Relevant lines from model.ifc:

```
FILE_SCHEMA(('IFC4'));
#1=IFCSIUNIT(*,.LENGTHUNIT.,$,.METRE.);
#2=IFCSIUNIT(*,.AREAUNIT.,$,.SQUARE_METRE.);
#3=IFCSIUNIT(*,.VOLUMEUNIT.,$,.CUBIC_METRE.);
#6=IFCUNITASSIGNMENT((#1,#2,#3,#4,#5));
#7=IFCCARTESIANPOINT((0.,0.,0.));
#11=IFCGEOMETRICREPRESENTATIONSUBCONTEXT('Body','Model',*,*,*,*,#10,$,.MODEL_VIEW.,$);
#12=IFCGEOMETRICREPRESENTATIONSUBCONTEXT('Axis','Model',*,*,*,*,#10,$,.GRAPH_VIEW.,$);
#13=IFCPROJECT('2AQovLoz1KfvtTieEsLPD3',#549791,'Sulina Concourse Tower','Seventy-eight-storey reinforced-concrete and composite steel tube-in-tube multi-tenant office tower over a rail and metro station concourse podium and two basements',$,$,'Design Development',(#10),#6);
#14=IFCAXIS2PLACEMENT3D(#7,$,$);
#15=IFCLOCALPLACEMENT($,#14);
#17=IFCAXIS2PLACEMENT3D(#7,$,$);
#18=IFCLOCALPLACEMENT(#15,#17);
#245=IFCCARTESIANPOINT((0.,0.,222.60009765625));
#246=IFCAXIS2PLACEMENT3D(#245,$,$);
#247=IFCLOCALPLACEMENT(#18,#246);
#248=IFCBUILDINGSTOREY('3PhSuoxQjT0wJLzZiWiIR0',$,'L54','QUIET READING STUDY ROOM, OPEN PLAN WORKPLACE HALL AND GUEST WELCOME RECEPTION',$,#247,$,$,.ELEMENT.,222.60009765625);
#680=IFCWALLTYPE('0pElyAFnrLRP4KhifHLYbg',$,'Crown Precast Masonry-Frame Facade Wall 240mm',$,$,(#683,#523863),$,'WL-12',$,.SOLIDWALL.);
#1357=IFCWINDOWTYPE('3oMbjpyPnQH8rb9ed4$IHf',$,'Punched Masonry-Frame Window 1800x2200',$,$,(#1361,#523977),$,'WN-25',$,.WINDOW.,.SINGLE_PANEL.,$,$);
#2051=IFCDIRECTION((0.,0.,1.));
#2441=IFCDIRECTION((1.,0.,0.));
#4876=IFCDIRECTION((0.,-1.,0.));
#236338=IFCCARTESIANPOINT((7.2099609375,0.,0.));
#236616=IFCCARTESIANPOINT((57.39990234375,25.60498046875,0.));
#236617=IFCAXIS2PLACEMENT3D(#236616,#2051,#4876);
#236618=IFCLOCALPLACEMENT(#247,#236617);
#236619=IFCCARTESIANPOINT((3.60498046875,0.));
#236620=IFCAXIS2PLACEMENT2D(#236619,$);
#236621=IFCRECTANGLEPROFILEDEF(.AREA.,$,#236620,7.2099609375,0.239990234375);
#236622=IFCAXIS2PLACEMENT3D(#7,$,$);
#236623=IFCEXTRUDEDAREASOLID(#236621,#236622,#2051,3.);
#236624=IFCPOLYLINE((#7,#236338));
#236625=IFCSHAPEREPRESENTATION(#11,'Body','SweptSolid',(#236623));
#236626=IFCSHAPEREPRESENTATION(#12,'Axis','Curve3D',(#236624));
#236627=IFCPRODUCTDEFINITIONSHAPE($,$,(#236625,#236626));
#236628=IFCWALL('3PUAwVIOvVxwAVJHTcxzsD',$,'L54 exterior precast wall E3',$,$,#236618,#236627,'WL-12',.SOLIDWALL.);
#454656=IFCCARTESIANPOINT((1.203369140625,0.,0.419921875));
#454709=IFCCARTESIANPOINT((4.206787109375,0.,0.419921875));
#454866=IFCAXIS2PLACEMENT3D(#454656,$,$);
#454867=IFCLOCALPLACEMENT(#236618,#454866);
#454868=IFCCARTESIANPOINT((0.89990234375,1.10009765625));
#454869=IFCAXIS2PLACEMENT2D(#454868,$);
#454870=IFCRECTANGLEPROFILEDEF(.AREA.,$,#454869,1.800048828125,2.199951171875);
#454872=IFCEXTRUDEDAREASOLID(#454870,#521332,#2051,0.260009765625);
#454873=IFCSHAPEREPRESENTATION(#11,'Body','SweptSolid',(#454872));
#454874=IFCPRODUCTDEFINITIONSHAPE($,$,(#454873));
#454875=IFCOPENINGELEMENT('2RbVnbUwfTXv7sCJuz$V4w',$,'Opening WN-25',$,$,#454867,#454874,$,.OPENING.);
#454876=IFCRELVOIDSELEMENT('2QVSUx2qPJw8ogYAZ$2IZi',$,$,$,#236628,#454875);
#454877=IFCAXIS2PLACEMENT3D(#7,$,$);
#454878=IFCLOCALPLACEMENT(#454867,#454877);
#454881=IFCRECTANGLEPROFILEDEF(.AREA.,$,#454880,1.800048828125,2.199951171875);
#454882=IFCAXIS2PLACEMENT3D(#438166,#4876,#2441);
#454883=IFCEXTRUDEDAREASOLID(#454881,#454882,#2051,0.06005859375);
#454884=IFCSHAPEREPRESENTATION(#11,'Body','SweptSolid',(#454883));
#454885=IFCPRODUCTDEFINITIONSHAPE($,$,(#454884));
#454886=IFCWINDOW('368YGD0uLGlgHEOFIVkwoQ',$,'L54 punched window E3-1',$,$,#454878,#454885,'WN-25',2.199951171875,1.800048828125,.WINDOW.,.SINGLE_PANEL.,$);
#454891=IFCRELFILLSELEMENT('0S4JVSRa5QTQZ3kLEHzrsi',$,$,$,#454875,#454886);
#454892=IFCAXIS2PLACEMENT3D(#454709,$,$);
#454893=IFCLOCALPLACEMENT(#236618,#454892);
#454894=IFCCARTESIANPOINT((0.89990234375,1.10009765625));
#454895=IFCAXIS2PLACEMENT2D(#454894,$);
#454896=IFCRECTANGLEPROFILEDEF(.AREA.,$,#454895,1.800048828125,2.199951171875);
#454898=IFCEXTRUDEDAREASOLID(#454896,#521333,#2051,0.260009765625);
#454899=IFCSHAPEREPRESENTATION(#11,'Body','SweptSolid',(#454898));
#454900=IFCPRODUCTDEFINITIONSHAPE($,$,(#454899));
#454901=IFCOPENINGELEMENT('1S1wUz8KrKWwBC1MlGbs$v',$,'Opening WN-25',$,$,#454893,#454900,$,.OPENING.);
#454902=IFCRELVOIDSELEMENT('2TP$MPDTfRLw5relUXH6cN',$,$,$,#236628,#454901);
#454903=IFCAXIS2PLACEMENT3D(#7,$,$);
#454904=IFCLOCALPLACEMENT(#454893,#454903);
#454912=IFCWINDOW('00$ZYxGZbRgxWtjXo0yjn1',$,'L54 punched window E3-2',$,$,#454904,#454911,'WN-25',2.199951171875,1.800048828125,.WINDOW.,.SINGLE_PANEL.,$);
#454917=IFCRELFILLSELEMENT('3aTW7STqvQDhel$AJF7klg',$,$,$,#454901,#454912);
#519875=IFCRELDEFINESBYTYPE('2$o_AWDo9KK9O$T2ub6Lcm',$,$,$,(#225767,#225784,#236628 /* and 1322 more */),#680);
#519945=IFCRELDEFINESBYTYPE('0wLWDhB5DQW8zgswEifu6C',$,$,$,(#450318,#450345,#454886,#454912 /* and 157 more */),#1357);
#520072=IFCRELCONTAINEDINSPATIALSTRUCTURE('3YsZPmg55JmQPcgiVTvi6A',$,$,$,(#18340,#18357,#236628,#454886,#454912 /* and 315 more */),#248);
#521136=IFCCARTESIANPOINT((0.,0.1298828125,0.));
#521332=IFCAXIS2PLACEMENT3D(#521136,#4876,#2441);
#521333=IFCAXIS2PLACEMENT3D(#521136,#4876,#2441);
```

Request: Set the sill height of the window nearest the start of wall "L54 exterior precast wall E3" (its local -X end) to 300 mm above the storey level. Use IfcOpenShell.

```python
import numpy as np
import ifcopenshell
import ifcopenshell.api.geometry
import ifcopenshell.geom
import ifcopenshell.util.element
import ifcopenshell.util.placement
import ifcopenshell.util.shape
import ifcopenshell.util.unit

model = ifcopenshell.open("model.ifc")
unit_scale = ifcopenshell.util.unit.calculate_unit_scale(model)

window = model.by_guid("368YGD0uLGlgHEOFIVkwoQ")
opening = window.FillsVoids[0].RelatingOpeningElement
storey = ifcopenshell.util.element.get_container(window, ifc_class="IfcBuildingStorey")
level = ifcopenshell.util.placement.get_local_placement(storey.ObjectPlacement)[2, 3]

# The opening's origin need not be at the sill, so measure its lowest point.
shape = ifcopenshell.geom.create_shape(ifcopenshell.geom.settings(), opening)
bottom = ifcopenshell.util.shape.get_shape_bottom_elevation(shape, shape.geometry) / unit_scale
dz = level + 0.3 / unit_scale - bottom

shift = np.array([0.0, 0.0, dz])
# The window is placed relative to its opening, so it follows when the opening moves.
matrix = ifcopenshell.util.placement.get_local_placement(opening.ObjectPlacement)
matrix[:3, 3] += shift
ifcopenshell.api.geometry.edit_object_placement(
    model, product=opening, matrix=matrix, is_si=False, should_transform_children=True
)

print(f"moved by {dz * unit_scale:+.3f} m")

model.write("model_edited.ifc")
```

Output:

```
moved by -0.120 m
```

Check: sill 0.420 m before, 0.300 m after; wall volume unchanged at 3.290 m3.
